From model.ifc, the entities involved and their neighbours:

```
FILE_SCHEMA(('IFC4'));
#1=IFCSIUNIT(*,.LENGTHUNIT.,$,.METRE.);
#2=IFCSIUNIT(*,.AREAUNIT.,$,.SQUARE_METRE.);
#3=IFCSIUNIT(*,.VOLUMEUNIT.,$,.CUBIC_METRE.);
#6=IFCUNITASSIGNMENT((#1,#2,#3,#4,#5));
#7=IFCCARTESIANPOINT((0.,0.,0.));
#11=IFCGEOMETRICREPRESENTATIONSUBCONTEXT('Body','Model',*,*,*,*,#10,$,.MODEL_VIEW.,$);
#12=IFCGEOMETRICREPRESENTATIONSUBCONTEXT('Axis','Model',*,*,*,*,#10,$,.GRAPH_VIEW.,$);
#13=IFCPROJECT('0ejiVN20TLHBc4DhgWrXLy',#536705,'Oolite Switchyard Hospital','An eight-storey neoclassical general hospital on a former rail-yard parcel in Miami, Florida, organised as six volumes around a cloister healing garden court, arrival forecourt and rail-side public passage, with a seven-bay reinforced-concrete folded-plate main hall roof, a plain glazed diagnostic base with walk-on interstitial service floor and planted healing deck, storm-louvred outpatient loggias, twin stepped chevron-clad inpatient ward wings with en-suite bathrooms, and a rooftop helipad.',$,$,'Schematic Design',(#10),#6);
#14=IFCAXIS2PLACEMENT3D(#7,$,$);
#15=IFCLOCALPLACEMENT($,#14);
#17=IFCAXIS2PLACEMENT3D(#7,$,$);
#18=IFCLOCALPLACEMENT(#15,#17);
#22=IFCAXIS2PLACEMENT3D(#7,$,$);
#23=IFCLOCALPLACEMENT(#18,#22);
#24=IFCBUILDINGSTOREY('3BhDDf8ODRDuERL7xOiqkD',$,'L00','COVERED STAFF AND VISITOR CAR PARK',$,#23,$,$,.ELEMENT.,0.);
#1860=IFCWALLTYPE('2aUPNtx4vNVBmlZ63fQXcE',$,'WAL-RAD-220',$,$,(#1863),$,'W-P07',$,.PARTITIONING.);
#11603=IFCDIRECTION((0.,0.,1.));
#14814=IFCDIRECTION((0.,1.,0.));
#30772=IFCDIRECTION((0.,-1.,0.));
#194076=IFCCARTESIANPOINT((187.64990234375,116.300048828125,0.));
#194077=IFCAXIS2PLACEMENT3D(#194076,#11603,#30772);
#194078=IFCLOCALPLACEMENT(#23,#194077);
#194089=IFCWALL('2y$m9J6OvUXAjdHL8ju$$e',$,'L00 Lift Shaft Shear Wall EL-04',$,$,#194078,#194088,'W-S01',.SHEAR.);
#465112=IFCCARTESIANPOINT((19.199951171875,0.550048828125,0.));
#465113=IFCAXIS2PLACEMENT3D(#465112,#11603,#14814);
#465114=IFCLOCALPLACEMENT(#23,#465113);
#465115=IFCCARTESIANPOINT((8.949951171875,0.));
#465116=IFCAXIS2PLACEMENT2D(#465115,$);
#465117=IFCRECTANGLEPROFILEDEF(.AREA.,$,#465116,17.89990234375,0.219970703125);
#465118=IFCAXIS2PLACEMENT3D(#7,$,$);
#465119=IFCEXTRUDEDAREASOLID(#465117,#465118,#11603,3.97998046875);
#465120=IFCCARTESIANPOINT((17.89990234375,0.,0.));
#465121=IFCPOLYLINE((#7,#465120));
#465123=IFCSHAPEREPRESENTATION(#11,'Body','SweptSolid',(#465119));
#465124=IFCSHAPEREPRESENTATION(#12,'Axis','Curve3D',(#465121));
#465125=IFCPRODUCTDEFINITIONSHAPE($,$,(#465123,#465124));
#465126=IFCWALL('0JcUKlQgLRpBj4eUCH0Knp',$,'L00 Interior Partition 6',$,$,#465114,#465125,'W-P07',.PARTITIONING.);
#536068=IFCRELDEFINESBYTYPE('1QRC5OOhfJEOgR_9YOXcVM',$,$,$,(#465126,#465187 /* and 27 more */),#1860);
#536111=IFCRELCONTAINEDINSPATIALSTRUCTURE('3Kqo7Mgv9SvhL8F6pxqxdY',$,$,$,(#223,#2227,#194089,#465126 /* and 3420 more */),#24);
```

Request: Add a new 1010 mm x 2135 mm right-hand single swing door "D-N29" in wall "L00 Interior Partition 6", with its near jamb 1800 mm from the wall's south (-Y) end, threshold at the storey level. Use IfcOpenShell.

```python
import numpy as np
import ifcopenshell
import ifcopenshell.api.feature
import ifcopenshell.api.geometry
import ifcopenshell.api.root
import ifcopenshell.api.spatial
import ifcopenshell.geom
import ifcopenshell.util.element
import ifcopenshell.util.placement
import ifcopenshell.util.representation
import ifcopenshell.util.shape
import ifcopenshell.util.unit

model = ifcopenshell.open("model.ifc")
unit_scale = ifcopenshell.util.unit.calculate_unit_scale(model)
settings = ifcopenshell.geom.settings()


def volume(element):
    """Net volume in cubic metres, openings subtracted."""
    shape = ifcopenshell.geom.create_shape(settings, element)
    return ifcopenshell.util.shape.get_volume(shape.geometry)


wall = model.by_guid("0JcUKlQgLRpBj4eUCH0Knp")
storey = ifcopenshell.util.element.get_container(wall, ifc_class="IfcBuildingStorey")
context = ifcopenshell.util.representation.get_context(model, "Model", "Body", "MODEL_VIEW")
before = volume(wall)

width, height, from_end, sill = 1.01, 2.135, 1.8, 0.0  # metres

# The wall runs along its own X axis, and the end named is its -X end.
wall_shape = ifcopenshell.geom.create_shape(settings, wall)
x, y, z = ifcopenshell.util.shape.get_vertices(wall_shape.geometry).T
start = x.min() + from_end
face, thickness = float(y.min()), float(y.max() - y.min())
wall_matrix = ifcopenshell.util.placement.get_local_placement(wall.ObjectPlacement)
level = ifcopenshell.util.placement.get_local_placement(storey.ObjectPlacement)[2, 3]


def in_wall(x, y):
    """Placement at x, y metres in the wall's axes, at sill height."""
    matrix = wall_matrix.copy()
    matrix[:, 3] = wall_matrix @ np.array([x / unit_scale, y / unit_scale, 0.0, 1.0])
    matrix[2, 3] = level + sill / unit_scale
    return matrix


# Opening: a box that overshoots both wall faces by 50 mm.
opening = ifcopenshell.api.root.create_entity(model, ifc_class="IfcOpeningElement", predefined_type="OPENING")
box = ifcopenshell.api.geometry.add_wall_representation(
    model, context=context, length=width, height=height, thickness=thickness + 0.1
)
ifcopenshell.api.geometry.assign_representation(model, product=opening, representation=box)
ifcopenshell.api.geometry.edit_object_placement(model, product=opening, matrix=in_wall(start, face - 0.05), is_si=False)
ifcopenshell.api.feature.add_feature(model, feature=opening, element=wall)

door = ifcopenshell.api.root.create_entity(model, ifc_class="IfcDoor", name="D-N29", predefined_type="DOOR")
door.OverallWidth, door.OverallHeight = width / unit_scale, height / unit_scale
door.OperationType = "SINGLE_SWING_RIGHT"
body = ifcopenshell.api.geometry.add_door_representation(
    model,
    context=context,
    overall_width=door.OverallWidth,
    overall_height=door.OverallHeight,
    operation_type="SINGLE_SWING_RIGHT",
    lining_properties={"LiningDepth": thickness / unit_scale, "ThresholdDepth": thickness / unit_scale},
)
ifcopenshell.api.geometry.assign_representation(model, product=door, representation=body)
ifcopenshell.api.spatial.assign_container(model, products=[door], relating_structure=storey)
ifcopenshell.api.feature.add_filling(model, opening=opening, element=door)

# The lining spans the wall, so the door starts at the wall face.
ifcopenshell.api.geometry.edit_object_placement(model, product=door, matrix=in_wall(start, face), is_si=False)

after = volume(wall)

print(f"wall volume {before:.3f} -> {after:.3f} m3")

model.write("model_updated.ifc")
```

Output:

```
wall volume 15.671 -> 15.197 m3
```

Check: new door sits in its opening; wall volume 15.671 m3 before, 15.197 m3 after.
